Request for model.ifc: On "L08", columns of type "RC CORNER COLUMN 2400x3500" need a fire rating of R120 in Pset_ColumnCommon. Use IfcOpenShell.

First a look at what the model holds.

```python
import ifcopenshell
import ifcopenshell.util.element

model = ifcopenshell.open("model.ifc")
print(model.schema)
storey = next(s for s in model.by_type("IfcBuildingStorey") if s.Name == "L08")
columns = [e for e in ifcopenshell.util.element.get_decomposition(storey) if e.is_a("IfcColumn")]
seen = {}
for e in columns:
    element_type = ifcopenshell.util.element.get_type(e)
    key = (element_type.Name if element_type != e and element_type else None, ifcopenshell.util.element.get_pset(e, "Pset_ColumnCommon", "FireRating"))
    seen[key] = seen.get(key, 0) + 1
for (name, value), count in sorted(seen.items(), key=str):
    print(count, "x", name, "|", value)
```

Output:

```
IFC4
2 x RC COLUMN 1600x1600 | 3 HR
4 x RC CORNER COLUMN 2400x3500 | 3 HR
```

```python
import ifcopenshell
import ifcopenshell.api.pset
import ifcopenshell.util.element

model = ifcopenshell.open("model.ifc")

storey = next(s for s in model.by_type("IfcBuildingStorey") if s.Name == "L08")
columns = [e for e in ifcopenshell.util.element.get_decomposition(storey) if e.is_a("IfcColumn")]

count = 0
for e in columns:
    element_type = ifcopenshell.util.element.get_type(e)
    if element_type in (None, e) or element_type.Name != "RC CORNER COLUMN 2400x3500":
        continue
    found = ifcopenshell.util.element.get_pset(e, "Pset_ColumnCommon", should_inherit=False)
    if found:
        pset = model.by_id(found["id"])
        if len(ifcopenshell.util.element.get_elements_by_pset(pset)) > 1:
            pset = ifcopenshell.api.pset.unshare_pset(model, products=[e], pset=pset)[0]
    else:
        pset = ifcopenshell.api.pset.add_pset(model, product=e, name="Pset_ColumnCommon")
    ifcopenshell.api.pset.edit_pset(model, pset=pset, properties={"FireRating": "R120"})
    count += 1

print(count, "columns updated")

model.write("model_v2.ifc")
```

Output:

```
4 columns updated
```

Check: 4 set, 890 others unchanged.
